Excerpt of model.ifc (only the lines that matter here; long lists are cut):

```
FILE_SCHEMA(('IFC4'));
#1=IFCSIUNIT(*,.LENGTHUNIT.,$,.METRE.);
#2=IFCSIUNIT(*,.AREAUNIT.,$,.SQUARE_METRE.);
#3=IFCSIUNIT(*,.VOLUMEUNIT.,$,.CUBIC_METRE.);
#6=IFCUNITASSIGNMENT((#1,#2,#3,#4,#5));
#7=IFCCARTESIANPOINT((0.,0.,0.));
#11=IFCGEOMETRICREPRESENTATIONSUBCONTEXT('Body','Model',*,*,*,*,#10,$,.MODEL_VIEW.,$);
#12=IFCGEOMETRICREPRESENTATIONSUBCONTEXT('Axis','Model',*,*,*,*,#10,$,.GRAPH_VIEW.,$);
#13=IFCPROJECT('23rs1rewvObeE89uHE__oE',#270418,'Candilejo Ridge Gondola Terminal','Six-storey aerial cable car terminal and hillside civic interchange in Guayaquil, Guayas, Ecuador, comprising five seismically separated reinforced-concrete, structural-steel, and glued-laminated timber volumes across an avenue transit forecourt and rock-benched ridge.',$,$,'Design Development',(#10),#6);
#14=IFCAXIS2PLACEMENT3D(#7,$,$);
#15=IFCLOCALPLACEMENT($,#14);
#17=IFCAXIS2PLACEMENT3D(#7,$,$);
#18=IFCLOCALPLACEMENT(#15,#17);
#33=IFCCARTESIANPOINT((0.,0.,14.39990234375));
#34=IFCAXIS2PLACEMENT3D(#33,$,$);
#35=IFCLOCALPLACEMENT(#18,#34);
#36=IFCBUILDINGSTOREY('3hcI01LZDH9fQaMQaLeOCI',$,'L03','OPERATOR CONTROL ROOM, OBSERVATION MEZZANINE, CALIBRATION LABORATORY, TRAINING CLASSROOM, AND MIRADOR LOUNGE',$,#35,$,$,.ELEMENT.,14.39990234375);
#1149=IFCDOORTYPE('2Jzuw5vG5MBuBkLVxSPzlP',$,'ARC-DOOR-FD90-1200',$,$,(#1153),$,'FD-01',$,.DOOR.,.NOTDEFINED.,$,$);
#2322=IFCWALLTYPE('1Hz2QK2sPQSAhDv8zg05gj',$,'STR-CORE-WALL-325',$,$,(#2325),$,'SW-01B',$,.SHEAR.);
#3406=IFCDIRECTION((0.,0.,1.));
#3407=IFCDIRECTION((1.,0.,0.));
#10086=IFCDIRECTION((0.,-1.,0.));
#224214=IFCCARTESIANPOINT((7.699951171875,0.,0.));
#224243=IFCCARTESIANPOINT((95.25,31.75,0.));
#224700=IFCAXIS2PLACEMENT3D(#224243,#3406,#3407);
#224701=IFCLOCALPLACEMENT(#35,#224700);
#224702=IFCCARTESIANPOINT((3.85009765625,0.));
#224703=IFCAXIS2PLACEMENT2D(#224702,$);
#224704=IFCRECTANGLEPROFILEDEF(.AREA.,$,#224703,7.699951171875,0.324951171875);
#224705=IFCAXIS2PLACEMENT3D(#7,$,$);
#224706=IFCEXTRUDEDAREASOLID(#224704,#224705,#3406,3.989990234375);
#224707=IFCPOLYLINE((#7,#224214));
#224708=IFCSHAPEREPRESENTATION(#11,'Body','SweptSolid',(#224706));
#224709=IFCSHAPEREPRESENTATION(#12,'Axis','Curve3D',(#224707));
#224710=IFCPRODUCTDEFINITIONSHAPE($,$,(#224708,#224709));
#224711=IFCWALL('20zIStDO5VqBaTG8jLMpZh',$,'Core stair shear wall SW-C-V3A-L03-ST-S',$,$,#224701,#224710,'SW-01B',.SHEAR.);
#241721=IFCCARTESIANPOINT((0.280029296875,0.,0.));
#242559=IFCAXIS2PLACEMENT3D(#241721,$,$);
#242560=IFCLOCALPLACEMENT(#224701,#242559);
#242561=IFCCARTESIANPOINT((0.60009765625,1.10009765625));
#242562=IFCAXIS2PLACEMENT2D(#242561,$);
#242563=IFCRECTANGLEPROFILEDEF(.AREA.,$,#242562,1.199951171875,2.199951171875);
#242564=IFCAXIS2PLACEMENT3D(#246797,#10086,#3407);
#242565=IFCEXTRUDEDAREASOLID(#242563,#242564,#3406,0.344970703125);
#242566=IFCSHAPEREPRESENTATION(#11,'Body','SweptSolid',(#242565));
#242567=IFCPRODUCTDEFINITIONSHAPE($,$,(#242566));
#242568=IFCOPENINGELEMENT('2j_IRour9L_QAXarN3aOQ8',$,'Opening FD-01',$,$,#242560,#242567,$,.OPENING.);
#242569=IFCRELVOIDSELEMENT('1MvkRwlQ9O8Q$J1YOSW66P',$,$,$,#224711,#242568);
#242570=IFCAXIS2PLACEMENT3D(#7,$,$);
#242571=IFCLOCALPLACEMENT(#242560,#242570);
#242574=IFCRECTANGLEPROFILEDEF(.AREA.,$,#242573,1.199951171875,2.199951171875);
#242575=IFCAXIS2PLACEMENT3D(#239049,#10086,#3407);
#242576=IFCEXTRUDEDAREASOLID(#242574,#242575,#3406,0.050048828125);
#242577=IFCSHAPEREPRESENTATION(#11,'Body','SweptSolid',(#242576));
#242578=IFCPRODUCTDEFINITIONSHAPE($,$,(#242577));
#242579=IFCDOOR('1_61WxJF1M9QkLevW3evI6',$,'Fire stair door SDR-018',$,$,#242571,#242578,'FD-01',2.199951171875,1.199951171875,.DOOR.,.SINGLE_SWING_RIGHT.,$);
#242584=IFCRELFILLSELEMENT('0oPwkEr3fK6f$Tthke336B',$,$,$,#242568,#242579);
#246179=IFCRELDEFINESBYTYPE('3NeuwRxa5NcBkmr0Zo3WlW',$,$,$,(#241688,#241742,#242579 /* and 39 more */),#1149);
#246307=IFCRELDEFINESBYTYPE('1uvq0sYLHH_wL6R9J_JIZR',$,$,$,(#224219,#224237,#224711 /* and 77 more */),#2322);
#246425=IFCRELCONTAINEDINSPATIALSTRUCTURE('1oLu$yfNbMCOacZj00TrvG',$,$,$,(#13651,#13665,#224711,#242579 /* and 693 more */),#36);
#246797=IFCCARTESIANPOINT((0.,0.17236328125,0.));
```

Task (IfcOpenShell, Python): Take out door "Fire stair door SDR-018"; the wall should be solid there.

```python
import ifcopenshell
import ifcopenshell.api.feature
import ifcopenshell.api.root
import ifcopenshell.geom
import ifcopenshell.util.shape

model = ifcopenshell.open("model.ifc")
settings = ifcopenshell.geom.settings()


def volume(element):
    """Net volume in cubic metres, openings subtracted."""
    shape = ifcopenshell.geom.create_shape(settings, element)
    return ifcopenshell.util.shape.get_volume(shape.geometry)


door = model.by_guid("1_61WxJF1M9QkLevW3evI6")
opening = door.FillsVoids[0].RelatingOpeningElement
wall = opening.VoidsElements[0].RelatingBuildingElement
before = volume(wall)

ifcopenshell.api.root.remove_product(model, product=door)
ifcopenshell.api.feature.remove_feature(model, feature=opening)

after = volume(wall)

print(f"wall volume {before:.3f} -> {after:.3f} m3")

model.write("model-out.ifc")
```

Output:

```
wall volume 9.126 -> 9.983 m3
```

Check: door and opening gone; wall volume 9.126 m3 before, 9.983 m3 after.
